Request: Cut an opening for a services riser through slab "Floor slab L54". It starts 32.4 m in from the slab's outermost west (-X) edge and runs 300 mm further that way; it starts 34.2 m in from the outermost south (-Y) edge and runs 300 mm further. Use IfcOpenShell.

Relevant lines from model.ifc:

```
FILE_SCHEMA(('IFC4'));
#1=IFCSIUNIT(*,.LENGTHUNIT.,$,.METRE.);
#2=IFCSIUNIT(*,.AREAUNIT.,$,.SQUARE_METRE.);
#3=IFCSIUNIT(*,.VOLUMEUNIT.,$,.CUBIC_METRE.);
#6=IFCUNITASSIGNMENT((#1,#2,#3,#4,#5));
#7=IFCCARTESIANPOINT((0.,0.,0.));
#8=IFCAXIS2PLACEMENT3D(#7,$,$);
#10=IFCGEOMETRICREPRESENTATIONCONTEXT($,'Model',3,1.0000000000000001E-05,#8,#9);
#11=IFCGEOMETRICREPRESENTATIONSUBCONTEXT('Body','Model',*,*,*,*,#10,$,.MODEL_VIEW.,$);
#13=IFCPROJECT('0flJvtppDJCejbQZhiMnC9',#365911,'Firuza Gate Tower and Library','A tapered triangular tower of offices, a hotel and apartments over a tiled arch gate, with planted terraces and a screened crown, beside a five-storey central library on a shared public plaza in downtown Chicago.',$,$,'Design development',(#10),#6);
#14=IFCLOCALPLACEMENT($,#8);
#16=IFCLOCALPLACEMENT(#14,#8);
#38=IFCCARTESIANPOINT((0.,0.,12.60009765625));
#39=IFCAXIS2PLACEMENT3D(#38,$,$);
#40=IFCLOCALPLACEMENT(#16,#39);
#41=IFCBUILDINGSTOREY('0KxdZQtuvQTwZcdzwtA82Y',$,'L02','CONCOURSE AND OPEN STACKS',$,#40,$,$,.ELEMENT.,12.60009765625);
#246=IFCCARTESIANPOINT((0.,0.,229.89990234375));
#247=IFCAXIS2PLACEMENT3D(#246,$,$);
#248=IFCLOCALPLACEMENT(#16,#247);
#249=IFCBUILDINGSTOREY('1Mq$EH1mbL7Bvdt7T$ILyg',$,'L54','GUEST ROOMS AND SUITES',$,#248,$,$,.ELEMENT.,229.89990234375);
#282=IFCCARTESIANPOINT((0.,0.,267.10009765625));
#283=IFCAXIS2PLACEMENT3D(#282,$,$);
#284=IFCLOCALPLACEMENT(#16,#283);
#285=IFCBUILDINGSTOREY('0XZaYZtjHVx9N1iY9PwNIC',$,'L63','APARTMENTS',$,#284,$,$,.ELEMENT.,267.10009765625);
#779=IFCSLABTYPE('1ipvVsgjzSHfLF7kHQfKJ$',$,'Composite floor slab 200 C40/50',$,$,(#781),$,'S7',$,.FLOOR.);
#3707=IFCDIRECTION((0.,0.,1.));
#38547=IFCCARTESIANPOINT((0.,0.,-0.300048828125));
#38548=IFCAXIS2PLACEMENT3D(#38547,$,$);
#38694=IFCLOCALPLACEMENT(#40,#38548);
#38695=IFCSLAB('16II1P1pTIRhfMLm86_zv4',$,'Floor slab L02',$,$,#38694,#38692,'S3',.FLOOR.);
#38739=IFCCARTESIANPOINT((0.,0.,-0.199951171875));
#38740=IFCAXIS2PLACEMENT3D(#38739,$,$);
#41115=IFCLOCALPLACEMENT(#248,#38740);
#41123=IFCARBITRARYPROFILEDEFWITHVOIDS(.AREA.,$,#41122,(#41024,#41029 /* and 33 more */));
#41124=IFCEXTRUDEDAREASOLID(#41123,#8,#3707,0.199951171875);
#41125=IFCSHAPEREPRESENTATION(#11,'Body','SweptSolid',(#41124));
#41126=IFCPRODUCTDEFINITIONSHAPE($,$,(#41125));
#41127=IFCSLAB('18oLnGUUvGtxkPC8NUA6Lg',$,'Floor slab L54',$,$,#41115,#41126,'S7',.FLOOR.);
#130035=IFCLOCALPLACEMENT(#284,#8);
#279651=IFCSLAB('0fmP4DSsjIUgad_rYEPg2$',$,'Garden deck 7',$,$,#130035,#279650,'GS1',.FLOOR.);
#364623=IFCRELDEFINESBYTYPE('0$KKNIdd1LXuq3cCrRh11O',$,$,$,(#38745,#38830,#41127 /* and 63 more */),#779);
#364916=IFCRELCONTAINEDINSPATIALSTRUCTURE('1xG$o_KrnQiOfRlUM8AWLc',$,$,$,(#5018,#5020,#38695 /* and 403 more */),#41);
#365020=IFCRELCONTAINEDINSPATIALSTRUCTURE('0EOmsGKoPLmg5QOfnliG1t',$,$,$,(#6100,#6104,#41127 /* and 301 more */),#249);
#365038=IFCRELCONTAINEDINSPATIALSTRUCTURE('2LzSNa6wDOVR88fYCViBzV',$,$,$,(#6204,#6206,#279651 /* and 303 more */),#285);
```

```python
import numpy as np
import ifcopenshell
import ifcopenshell.api.feature
import ifcopenshell.api.geometry
import ifcopenshell.api.root
import ifcopenshell.geom
import ifcopenshell.util.placement
import ifcopenshell.util.representation
import ifcopenshell.util.shape
import ifcopenshell.util.unit

model = ifcopenshell.open("model.ifc")
unit_scale = ifcopenshell.util.unit.calculate_unit_scale(model)
settings = ifcopenshell.geom.settings()


def volume(element):
    """Net volume in cubic metres, openings subtracted."""
    shape = ifcopenshell.geom.create_shape(settings, element)
    return ifcopenshell.util.shape.get_volume(shape.geometry)


slab = model.by_id(41127)
before = volume(slab)

# Extent in the slab's own axes, in metres. The edges named are its -X and -Y sides.
slab_shape = ifcopenshell.geom.create_shape(settings, slab)
vertices = ifcopenshell.util.shape.get_vertices(slab_shape.geometry)
x_min, y_min, bottom = vertices.min(axis=0)
top = vertices[:, 2].max()

opening = ifcopenshell.api.root.create_entity(model, ifc_class="IfcOpeningElement", name="Services riser opening", predefined_type="OPENING")
context = ifcopenshell.util.representation.get_context(model, "Model", "Body", "MODEL_VIEW")
width, depth = 0.3, 0.3
outline = [(0.0, 0.0), (width, 0.0), (width, depth), (0.0, depth), (0.0, 0.0)]
# Overshoot both faces by 50 mm so the cut is clean.
shape = ifcopenshell.api.geometry.add_slab_representation(
    model, context=context, depth=top - bottom + 0.1, polyline=outline
)
ifcopenshell.api.geometry.assign_representation(model, product=opening, representation=shape)

matrix = ifcopenshell.util.placement.get_local_placement(slab.ObjectPlacement)
matrix[:, 3] = matrix @ np.append(np.array([x_min + 32.4, y_min + 34.2, bottom - 0.05]) / unit_scale, 1.0)
ifcopenshell.api.geometry.edit_object_placement(model, product=opening, matrix=matrix, is_si=False)
ifcopenshell.api.feature.add_feature(model, feature=opening, element=slab)

after = volume(slab)

print(f"slab volume {before:.3f} -> {after:.3f} m3")

model.write("model_v2.ifc")
```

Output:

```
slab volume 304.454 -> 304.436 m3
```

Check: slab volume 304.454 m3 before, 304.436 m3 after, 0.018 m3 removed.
